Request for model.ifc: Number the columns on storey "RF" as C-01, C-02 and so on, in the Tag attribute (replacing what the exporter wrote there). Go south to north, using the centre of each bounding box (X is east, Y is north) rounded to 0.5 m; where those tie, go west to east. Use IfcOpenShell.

First a look at what the model holds.

```python
import ifcopenshell
import ifcopenshell.util.element
import ifcopenshell.util.placement

model = ifcopenshell.open("model.ifc")
print(model.schema)
storey = next(s for s in model.by_type("IfcBuildingStorey") if s.Name == "RF")
columns = [e for e in ifcopenshell.util.element.get_decomposition(storey) if e.is_a("IfcColumn")]
for e in sorted(columns, key=lambda e: e.id()):
    origin = ifcopenshell.util.placement.get_local_placement(e.ObjectPlacement)[:3, 3]
    print(e.id(), e.Tag, e.Name, origin.round(2) + 0.0, sep=" | ")
```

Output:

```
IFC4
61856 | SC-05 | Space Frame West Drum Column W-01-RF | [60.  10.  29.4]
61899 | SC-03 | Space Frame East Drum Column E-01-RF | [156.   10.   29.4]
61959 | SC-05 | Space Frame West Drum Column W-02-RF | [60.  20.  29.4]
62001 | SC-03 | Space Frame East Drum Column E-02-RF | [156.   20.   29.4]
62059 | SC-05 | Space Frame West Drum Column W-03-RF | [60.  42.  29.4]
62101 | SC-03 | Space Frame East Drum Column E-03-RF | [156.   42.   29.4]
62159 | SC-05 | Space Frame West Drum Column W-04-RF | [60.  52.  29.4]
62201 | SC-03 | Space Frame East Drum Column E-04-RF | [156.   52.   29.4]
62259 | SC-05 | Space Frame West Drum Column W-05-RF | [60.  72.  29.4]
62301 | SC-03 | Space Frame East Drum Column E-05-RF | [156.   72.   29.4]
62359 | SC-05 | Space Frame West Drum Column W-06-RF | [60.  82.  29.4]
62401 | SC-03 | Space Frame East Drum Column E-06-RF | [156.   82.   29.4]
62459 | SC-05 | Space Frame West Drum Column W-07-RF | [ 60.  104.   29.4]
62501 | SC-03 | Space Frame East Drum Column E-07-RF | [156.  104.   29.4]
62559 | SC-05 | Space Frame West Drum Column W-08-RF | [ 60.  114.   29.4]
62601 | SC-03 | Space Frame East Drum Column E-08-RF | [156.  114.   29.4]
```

```python
import ifcopenshell
import ifcopenshell.geom
import ifcopenshell.util.element
import ifcopenshell.util.shape

model = ifcopenshell.open("model.ifc")
settings = ifcopenshell.geom.settings()
settings.set("use-world-coords", True)


def centre(element):
    shape = ifcopenshell.geom.create_shape(settings, element)
    return ifcopenshell.util.shape.get_bbox_centroid(shape.geometry)


storey = next(s for s in model.by_type("IfcBuildingStorey") if s.Name == "RF")
columns = [e for e in ifcopenshell.util.element.get_decomposition(storey) if e.is_a("IfcColumn")]

# Insertion points can sit at a corner or the storey origin, so sort by the geometry (in metres).
centres = {e: centre(e) for e in columns}
columns.sort(key=lambda e: (round(centres[e][1] / 0.5), centres[e][0]))

for i, e in enumerate(columns, start=1):
    number = f"C-{i:02d}"
    e.Tag = number
    print(e.id(), number)

model.write("model_updated.ifc")
```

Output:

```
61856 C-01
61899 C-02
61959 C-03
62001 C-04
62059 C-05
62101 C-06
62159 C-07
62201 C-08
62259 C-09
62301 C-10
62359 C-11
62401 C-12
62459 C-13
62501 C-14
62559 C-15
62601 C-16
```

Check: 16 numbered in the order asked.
